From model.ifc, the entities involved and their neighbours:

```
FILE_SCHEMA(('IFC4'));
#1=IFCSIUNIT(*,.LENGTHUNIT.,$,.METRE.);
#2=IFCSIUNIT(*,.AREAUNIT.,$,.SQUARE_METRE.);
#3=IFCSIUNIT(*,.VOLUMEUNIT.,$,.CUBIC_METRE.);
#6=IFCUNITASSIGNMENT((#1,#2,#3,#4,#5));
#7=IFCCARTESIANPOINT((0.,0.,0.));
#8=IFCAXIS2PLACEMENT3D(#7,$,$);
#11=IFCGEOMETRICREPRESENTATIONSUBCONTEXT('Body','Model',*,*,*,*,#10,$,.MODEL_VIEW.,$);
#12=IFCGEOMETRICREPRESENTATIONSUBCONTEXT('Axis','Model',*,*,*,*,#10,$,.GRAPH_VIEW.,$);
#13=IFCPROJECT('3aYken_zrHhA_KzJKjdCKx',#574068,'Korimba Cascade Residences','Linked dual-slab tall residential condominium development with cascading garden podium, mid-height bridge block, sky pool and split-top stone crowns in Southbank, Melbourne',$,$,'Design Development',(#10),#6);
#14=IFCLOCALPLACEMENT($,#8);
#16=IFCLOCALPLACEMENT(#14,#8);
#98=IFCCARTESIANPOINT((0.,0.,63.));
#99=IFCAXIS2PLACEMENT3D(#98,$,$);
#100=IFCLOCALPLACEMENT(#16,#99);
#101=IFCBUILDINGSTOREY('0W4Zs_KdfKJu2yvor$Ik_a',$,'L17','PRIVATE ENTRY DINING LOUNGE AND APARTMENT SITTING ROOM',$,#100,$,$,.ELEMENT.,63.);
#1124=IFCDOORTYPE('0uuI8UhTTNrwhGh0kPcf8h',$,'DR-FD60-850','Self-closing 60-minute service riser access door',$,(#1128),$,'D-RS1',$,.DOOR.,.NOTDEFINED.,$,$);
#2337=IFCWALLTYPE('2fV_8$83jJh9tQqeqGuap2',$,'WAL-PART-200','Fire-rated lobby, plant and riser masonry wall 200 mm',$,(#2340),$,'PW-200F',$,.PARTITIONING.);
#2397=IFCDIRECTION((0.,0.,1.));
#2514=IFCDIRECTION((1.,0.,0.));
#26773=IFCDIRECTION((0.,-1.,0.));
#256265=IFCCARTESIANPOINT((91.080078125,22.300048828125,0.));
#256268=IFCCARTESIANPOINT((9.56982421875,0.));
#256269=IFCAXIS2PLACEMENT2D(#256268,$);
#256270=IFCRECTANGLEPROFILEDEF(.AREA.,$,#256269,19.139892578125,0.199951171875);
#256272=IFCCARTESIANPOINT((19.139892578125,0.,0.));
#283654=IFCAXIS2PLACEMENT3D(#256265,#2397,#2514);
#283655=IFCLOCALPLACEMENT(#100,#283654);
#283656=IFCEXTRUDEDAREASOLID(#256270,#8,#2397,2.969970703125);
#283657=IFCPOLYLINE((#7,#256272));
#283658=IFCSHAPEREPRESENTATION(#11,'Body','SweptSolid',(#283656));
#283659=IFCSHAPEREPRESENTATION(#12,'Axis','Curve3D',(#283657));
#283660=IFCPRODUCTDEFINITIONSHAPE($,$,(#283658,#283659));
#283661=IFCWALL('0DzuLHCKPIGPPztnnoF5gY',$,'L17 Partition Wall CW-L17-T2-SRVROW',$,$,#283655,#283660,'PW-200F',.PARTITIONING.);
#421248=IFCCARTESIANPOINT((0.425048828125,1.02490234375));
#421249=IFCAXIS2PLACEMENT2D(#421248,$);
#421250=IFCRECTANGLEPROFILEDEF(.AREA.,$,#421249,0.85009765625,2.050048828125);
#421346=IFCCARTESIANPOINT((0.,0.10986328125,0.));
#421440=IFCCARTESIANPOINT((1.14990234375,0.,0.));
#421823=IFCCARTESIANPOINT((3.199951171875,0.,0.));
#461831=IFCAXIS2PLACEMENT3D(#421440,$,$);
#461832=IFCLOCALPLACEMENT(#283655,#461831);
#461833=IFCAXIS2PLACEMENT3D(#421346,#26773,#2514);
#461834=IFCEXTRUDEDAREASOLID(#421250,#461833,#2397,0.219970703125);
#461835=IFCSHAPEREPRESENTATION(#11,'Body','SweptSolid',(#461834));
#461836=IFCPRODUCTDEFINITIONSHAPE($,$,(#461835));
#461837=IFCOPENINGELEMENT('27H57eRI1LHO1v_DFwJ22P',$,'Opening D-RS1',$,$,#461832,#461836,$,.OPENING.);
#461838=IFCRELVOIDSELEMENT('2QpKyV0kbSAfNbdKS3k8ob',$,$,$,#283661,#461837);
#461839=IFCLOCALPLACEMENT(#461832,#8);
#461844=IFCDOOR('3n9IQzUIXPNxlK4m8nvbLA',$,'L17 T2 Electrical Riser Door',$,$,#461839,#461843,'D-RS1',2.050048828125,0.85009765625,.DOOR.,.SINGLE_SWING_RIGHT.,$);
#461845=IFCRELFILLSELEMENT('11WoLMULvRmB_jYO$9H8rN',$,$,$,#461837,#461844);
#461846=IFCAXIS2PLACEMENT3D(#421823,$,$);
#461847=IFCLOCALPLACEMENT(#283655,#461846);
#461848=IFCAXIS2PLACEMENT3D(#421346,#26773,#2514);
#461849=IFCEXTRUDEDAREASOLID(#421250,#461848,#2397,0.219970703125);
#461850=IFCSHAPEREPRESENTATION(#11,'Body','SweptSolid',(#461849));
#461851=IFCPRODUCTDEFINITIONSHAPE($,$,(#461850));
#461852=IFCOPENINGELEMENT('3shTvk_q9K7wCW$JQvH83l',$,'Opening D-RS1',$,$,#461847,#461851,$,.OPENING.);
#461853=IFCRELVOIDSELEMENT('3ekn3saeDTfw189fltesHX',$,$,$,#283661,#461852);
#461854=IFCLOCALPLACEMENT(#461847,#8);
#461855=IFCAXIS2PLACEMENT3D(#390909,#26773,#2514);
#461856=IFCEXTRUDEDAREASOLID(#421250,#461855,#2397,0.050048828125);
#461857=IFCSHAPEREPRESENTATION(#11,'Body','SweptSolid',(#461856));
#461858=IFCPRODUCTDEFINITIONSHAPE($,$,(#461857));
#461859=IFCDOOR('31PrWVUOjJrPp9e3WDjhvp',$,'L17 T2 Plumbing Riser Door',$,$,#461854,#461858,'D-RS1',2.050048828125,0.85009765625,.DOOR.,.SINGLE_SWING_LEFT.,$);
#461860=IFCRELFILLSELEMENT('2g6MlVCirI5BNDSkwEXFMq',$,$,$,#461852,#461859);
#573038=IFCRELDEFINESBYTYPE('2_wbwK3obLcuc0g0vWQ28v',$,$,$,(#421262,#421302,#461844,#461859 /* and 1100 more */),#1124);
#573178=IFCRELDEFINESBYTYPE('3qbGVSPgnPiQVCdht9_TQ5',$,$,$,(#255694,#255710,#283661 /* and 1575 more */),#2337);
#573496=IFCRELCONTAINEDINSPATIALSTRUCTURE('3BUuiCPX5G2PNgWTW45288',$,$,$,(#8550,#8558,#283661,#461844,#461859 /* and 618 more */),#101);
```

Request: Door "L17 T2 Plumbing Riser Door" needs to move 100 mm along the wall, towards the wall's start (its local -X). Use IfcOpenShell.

```python
import ifcopenshell
import ifcopenshell.api.geometry
import ifcopenshell.util.placement

model = ifcopenshell.open("model.ifc")

door = model.by_guid("31PrWVUOjJrPp9e3WDjhvp")
opening = door.FillsVoids[0].RelatingOpeningElement
wall = opening.VoidsElements[0].RelatingBuildingElement

wall_matrix = ifcopenshell.util.placement.get_local_placement(wall.ObjectPlacement)
shift = wall_matrix[:3, 0] * -0.1
before = ifcopenshell.util.placement.get_local_placement(door.ObjectPlacement)[:3, 3].copy()

# The door is placed relative to its opening, so it follows when the opening moves.
matrix = ifcopenshell.util.placement.get_local_placement(opening.ObjectPlacement)
matrix[:3, 3] += shift
ifcopenshell.api.geometry.edit_object_placement(
    model, product=opening, matrix=matrix, is_si=False, should_transform_children=True
)

after = ifcopenshell.util.placement.get_local_placement(door.ObjectPlacement)[:3, 3]
print("door moved by", (after - before).round(3) + 0.0)

model.write("model_v2.ifc")
```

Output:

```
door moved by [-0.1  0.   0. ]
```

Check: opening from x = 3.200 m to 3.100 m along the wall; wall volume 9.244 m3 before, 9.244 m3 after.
